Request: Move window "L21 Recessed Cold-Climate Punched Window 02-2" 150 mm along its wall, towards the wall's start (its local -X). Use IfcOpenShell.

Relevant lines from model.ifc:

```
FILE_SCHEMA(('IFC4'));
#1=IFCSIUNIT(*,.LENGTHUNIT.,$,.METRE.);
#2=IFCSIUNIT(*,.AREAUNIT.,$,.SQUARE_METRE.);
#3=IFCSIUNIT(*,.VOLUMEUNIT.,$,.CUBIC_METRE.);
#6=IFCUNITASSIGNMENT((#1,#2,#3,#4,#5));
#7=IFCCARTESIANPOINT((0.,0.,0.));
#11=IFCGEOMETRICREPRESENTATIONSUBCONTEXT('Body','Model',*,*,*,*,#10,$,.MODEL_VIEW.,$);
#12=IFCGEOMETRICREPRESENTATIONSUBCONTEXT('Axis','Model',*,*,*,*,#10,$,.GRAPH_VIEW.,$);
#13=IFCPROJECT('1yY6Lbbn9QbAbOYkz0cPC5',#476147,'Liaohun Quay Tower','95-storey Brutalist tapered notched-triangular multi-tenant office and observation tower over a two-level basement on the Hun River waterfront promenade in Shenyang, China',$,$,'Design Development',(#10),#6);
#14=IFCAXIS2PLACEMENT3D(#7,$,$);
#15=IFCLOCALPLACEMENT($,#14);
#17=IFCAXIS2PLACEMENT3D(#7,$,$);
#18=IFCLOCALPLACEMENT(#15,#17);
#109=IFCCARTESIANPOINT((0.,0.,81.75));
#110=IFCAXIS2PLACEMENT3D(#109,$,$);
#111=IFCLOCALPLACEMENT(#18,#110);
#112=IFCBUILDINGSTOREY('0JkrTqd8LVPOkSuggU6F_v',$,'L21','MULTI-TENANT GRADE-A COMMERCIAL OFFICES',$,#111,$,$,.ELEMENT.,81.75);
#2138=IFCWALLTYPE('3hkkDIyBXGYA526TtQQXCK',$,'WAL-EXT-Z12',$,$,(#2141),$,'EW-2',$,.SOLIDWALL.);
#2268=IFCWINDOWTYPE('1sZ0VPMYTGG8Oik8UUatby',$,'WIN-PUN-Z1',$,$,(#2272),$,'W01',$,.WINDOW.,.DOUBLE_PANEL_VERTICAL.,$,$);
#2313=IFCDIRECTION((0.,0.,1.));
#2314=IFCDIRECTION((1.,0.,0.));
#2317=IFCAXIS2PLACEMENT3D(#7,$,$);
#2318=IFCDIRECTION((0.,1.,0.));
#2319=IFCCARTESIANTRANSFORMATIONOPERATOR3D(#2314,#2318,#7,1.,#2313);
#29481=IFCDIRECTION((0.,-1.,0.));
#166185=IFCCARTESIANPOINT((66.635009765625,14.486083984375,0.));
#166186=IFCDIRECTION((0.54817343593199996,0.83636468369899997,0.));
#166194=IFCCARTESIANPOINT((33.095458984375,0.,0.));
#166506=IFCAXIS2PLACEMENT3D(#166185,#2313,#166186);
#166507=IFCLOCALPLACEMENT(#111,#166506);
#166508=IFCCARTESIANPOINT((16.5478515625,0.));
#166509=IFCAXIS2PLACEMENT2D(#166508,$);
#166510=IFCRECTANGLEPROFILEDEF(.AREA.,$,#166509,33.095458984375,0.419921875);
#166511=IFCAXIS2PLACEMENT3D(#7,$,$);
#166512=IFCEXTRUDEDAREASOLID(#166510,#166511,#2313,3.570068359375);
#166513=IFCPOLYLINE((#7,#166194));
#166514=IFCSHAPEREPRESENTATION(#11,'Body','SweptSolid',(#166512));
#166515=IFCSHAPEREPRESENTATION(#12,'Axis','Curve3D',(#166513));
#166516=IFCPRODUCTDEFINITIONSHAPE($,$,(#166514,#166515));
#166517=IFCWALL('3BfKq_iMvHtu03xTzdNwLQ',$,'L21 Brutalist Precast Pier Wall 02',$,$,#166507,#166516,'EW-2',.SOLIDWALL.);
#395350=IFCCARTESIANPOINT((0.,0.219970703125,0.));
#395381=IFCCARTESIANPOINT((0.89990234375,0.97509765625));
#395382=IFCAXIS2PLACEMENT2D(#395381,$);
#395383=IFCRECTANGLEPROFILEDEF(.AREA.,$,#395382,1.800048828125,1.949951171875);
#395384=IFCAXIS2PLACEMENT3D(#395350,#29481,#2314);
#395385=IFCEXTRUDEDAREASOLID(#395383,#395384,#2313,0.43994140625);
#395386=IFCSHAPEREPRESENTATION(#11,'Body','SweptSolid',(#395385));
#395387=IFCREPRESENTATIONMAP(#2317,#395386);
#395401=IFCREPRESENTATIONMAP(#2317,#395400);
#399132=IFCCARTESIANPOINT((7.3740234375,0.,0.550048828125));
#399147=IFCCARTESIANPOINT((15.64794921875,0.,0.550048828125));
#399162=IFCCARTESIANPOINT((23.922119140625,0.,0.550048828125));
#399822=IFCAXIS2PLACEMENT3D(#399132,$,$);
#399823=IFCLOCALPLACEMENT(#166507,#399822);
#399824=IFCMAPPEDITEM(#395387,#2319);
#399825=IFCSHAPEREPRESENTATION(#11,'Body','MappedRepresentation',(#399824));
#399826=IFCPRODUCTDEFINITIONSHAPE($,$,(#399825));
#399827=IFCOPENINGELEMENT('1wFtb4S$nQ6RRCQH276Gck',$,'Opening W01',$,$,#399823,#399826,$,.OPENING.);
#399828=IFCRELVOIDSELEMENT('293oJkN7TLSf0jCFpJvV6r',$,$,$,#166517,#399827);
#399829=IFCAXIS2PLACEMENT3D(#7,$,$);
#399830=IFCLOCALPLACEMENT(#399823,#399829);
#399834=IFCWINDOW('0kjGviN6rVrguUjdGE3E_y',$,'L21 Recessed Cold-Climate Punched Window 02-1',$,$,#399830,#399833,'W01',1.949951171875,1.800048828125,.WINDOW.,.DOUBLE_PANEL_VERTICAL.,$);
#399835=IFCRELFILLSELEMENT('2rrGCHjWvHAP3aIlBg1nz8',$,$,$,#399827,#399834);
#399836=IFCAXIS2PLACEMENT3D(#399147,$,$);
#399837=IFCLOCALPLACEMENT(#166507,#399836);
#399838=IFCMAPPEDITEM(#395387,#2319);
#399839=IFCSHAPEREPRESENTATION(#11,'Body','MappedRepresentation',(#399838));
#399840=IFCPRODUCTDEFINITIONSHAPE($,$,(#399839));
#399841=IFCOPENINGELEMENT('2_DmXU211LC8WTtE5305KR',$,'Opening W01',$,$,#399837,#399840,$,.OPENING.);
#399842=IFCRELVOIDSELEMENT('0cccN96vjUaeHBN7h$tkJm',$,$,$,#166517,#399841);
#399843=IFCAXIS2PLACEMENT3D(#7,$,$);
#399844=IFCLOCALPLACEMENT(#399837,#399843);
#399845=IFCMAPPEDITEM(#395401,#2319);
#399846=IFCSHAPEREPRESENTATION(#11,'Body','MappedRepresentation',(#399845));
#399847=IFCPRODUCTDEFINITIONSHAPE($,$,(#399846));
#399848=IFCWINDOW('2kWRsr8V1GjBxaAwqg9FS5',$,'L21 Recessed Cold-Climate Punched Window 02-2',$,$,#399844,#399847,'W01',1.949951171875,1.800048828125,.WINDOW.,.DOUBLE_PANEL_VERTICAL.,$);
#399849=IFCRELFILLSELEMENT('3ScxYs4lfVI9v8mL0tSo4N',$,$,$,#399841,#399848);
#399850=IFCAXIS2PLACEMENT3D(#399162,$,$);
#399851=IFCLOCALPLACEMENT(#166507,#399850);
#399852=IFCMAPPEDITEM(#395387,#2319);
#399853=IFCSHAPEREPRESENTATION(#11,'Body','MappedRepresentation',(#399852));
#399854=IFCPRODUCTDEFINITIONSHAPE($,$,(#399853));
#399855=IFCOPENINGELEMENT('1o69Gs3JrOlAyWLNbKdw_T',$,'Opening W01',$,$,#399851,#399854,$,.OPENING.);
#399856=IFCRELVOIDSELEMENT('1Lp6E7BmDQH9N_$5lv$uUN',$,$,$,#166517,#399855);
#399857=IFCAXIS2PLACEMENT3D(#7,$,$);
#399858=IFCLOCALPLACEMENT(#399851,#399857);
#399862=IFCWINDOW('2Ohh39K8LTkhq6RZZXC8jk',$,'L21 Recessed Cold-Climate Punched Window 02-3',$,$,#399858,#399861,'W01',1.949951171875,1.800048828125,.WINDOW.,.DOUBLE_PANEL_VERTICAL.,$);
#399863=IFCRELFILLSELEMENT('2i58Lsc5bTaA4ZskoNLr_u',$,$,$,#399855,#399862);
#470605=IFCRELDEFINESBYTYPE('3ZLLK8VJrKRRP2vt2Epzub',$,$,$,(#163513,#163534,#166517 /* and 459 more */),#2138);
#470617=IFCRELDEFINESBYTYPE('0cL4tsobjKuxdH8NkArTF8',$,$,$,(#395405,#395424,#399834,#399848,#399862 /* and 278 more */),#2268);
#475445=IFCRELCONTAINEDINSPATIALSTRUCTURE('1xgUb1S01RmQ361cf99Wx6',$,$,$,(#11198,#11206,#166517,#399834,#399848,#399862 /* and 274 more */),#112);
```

```python
import ifcopenshell
import ifcopenshell.api.geometry
import ifcopenshell.util.placement
import ifcopenshell.util.unit

model = ifcopenshell.open("model.ifc")
unit_scale = ifcopenshell.util.unit.calculate_unit_scale(model)

window = model.by_guid("2kWRsr8V1GjBxaAwqg9FS5")
opening = window.FillsVoids[0].RelatingOpeningElement
wall = opening.VoidsElements[0].RelatingBuildingElement

wall_matrix = ifcopenshell.util.placement.get_local_placement(wall.ObjectPlacement)
shift = wall_matrix[:3, 0] * -0.15 / unit_scale
before = ifcopenshell.util.placement.get_local_placement(window.ObjectPlacement)[:3, 3].copy()

# The window is placed relative to its opening, so it follows when the opening moves.
matrix = ifcopenshell.util.placement.get_local_placement(opening.ObjectPlacement)
matrix[:3, 3] += shift
ifcopenshell.api.geometry.edit_object_placement(
    model, product=opening, matrix=matrix, is_si=False, should_transform_children=True
)

after = ifcopenshell.util.placement.get_local_placement(window.ObjectPlacement)[:3, 3]
print("window moved by", (after - before).round(3) + 0.0)

model.write("model_edited.ifc")
```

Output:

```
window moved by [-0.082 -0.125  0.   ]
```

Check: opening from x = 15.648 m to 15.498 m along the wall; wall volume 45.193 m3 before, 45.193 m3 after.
